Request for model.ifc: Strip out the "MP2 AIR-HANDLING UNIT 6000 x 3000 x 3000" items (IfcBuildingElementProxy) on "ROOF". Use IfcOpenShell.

First a look at what the model holds.

```python
import ifcopenshell
import ifcopenshell.util.element

model = ifcopenshell.open("model.ifc")
print(model.schema)
storey = next(s for s in model.by_type("IfcBuildingStorey") if s.Name == "ROOF")
proxies = [e for e in ifcopenshell.util.element.get_decomposition(storey) if e.is_a("IfcBuildingElementProxy")]
seen = {}
for e in proxies:
    element_type = ifcopenshell.util.element.get_type(e)
    name = element_type.Name if element_type not in (None, e) else None
    seen[name] = seen.get(name, 0) + 1
for name, count in sorted(seen.items(), key=str):
    print(count, "x", name)
```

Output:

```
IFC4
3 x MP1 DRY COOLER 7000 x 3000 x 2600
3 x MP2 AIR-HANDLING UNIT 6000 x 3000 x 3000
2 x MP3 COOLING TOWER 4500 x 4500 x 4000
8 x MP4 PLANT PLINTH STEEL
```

```python
import ifcopenshell
import ifcopenshell.api.root
import ifcopenshell.util.element

model = ifcopenshell.open("model.ifc")

storey = next(s for s in model.by_type("IfcBuildingStorey") if s.Name == "ROOF")
proxies = [e for e in ifcopenshell.util.element.get_decomposition(storey) if e.is_a("IfcBuildingElementProxy")]
targets = [e for e in proxies if (t := ifcopenshell.util.element.get_type(e)) not in (None, e) and t.Name == "MP2 AIR-HANDLING UNIT 6000 x 3000 x 3000"]

for e in targets:
    ifcopenshell.api.root.remove_product(model, product=e)
print(len(targets), "removed")

model.write("model_edited.ifc")
```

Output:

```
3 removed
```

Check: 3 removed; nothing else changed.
